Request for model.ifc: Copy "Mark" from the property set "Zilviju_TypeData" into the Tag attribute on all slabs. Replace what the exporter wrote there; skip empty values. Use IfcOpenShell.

First a look at what the model holds.

```python
import ifcopenshell
import ifcopenshell.util.element

model = ifcopenshell.open("model.ifc")
print(model.schema)
slabs = model.by_type("IfcSlab")
print(len(slabs), "slabs")
for e in slabs[:8]:
    source = ifcopenshell.util.element.get_pset(e, "Zilviju_TypeData", "Mark")
    target = e.Tag
    print(e.id(), repr(source), repr(target), sep=" | ")
```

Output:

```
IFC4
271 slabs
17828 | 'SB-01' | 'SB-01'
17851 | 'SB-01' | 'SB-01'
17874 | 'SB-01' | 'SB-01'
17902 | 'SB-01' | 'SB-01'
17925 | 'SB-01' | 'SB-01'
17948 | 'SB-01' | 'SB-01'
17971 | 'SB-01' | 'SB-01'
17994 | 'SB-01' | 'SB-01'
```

```python
import ifcopenshell
import ifcopenshell.util.element

model = ifcopenshell.open("model.ifc")

count = 0
for e in model.by_type("IfcSlab"):
    value = ifcopenshell.util.element.get_pset(e, "Zilviju_TypeData", "Mark")
    current = e.Tag
    if not value or not value.strip() or current == value:
        continue
    e.Tag = value
    count += 1

print(count, "slabs updated")

model.write("model-out.ifc")
```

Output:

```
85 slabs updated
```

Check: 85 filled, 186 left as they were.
